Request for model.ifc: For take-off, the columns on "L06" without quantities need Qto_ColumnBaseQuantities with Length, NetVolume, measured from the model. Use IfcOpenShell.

First a look at what the model holds.

```python
import ifcopenshell
import ifcopenshell.util.element
import ifcopenshell.util.unit

model = ifcopenshell.open("model.ifc")
print(model.schema)
for unit_type in ("LENGTHUNIT", "AREAUNIT", "VOLUMEUNIT"):
    print(unit_type, ifcopenshell.util.unit.calculate_unit_scale(model, unit_type))
storey = next(s for s in model.by_type("IfcBuildingStorey") if s.Name == "L06")
columns = [e for e in ifcopenshell.util.element.get_decomposition(storey) if e.is_a("IfcColumn")]
for e in sorted(columns, key=lambda e: e.id()):
    print(e.id(), e.is_a(), e.Name, list(ifcopenshell.util.element.get_psets(e, qtos_only=True)), sep=" | ")
```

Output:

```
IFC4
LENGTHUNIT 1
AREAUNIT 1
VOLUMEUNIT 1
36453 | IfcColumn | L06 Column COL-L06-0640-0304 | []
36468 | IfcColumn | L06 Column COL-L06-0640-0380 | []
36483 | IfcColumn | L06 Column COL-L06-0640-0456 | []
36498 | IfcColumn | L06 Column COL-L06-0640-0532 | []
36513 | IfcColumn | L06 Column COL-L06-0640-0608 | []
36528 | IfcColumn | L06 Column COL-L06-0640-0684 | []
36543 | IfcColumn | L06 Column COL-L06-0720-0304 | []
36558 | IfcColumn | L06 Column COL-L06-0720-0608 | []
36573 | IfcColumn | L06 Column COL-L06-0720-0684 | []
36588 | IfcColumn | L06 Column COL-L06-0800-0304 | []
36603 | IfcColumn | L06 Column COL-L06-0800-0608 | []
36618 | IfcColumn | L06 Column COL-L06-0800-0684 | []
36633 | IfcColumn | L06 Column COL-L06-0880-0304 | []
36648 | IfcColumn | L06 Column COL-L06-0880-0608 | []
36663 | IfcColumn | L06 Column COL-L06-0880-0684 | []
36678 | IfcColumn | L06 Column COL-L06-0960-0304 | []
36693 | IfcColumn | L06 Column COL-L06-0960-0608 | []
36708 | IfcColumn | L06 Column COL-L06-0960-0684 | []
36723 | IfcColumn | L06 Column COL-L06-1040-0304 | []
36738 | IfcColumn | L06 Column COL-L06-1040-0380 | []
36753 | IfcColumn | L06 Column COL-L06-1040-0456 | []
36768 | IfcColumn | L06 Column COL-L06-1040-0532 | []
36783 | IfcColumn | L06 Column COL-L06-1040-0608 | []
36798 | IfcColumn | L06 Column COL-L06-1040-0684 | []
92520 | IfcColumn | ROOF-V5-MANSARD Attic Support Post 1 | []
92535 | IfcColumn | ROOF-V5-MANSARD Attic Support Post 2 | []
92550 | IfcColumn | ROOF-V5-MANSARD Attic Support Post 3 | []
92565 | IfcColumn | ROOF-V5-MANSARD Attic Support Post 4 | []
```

```python
import ifcopenshell
import ifcopenshell.api.pset
import ifcopenshell.geom
import ifcopenshell.util.element
import ifcopenshell.util.shape
import ifcopenshell.util.unit

model = ifcopenshell.open("model.ifc")
unit_scale = ifcopenshell.util.unit.calculate_unit_scale(model)
volume_scale = ifcopenshell.util.unit.calculate_unit_scale(model, "VOLUMEUNIT")
settings = ifcopenshell.geom.settings()

storey = next(s for s in model.by_type("IfcBuildingStorey") if s.Name == "L06")
columns = [e for e in ifcopenshell.util.element.get_decomposition(storey) if e.is_a("IfcColumn")]

for e in sorted(columns, key=lambda e: e.id()):
    if ifcopenshell.util.element.get_psets(e, qtos_only=True, should_inherit=False):
        continue
    # Geometry comes back in metres, in the element's own axes.
    shape = ifcopenshell.geom.create_shape(settings, e)
    values = {
        "Length": ifcopenshell.util.shape.get_z(shape.geometry) / unit_scale,
        "NetVolume": ifcopenshell.util.shape.get_volume(shape.geometry) / volume_scale,
    }
    qto = ifcopenshell.api.pset.add_qto(model, product=e, name="Qto_ColumnBaseQuantities")
    ifcopenshell.api.pset.edit_qto(model, qto=qto, properties=values)
    print(e.id(), {k: round(v, 3) for k, v in values.items()})

model.write("model_rev.ifc")
```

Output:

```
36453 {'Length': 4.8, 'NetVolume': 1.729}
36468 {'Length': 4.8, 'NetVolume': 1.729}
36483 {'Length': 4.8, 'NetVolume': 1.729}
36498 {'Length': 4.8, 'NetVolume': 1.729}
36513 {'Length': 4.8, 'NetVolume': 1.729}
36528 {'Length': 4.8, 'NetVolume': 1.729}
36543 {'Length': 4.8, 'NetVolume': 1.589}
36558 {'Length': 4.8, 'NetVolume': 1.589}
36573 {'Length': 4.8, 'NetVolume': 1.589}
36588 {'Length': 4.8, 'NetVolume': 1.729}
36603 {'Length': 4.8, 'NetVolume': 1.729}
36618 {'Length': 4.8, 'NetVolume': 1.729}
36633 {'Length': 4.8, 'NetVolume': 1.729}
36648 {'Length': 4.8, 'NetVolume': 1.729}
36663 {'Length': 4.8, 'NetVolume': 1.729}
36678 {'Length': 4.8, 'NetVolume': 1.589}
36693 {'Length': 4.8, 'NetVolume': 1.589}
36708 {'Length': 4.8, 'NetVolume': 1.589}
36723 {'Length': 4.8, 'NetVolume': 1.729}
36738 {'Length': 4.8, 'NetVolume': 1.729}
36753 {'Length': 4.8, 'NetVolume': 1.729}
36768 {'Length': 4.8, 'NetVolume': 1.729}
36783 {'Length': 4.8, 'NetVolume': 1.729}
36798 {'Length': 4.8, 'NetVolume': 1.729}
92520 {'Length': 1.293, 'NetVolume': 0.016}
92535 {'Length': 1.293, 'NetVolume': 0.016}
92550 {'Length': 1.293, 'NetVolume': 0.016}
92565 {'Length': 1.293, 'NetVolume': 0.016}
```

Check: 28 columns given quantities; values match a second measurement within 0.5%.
